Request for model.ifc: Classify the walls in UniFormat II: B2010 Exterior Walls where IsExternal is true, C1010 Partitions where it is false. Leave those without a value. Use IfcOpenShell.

First a look at what the model holds.

```python
import ifcopenshell
import ifcopenshell.util.element

model = ifcopenshell.open("model.ifc")
print(model.schema)
print("classifications:", [c.Name for c in model.by_type("IfcClassification")])
values = [ifcopenshell.util.element.get_pset(e, "Pset_WallCommon", "IsExternal") for e in model.by_type("IfcWall")]
for value in (True, False, None):
    print("IsExternal", value, values.count(value))
```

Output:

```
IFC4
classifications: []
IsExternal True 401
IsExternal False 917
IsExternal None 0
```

```python
import ifcopenshell
import ifcopenshell.api.classification
import ifcopenshell.util.element

model = ifcopenshell.open("model.ifc")

system = ifcopenshell.api.classification.add_classification(model, classification="UniFormat II")

walls = model.by_type("IfcWall")
external = {e: ifcopenshell.util.element.get_pset(e, "Pset_WallCommon", "IsExternal") for e in walls}
for flag, code, name in ((True, "B2010", "Exterior Walls"), (False, "C1010", "Partitions")):
    products = [e for e in walls if external[e] is flag]
    ifcopenshell.api.classification.add_reference(
        model, products=products, classification=system, identification=code, name=name
    )
    print(code, len(products))

model.write("model_updated.ifc")
```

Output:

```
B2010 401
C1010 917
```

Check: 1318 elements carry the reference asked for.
